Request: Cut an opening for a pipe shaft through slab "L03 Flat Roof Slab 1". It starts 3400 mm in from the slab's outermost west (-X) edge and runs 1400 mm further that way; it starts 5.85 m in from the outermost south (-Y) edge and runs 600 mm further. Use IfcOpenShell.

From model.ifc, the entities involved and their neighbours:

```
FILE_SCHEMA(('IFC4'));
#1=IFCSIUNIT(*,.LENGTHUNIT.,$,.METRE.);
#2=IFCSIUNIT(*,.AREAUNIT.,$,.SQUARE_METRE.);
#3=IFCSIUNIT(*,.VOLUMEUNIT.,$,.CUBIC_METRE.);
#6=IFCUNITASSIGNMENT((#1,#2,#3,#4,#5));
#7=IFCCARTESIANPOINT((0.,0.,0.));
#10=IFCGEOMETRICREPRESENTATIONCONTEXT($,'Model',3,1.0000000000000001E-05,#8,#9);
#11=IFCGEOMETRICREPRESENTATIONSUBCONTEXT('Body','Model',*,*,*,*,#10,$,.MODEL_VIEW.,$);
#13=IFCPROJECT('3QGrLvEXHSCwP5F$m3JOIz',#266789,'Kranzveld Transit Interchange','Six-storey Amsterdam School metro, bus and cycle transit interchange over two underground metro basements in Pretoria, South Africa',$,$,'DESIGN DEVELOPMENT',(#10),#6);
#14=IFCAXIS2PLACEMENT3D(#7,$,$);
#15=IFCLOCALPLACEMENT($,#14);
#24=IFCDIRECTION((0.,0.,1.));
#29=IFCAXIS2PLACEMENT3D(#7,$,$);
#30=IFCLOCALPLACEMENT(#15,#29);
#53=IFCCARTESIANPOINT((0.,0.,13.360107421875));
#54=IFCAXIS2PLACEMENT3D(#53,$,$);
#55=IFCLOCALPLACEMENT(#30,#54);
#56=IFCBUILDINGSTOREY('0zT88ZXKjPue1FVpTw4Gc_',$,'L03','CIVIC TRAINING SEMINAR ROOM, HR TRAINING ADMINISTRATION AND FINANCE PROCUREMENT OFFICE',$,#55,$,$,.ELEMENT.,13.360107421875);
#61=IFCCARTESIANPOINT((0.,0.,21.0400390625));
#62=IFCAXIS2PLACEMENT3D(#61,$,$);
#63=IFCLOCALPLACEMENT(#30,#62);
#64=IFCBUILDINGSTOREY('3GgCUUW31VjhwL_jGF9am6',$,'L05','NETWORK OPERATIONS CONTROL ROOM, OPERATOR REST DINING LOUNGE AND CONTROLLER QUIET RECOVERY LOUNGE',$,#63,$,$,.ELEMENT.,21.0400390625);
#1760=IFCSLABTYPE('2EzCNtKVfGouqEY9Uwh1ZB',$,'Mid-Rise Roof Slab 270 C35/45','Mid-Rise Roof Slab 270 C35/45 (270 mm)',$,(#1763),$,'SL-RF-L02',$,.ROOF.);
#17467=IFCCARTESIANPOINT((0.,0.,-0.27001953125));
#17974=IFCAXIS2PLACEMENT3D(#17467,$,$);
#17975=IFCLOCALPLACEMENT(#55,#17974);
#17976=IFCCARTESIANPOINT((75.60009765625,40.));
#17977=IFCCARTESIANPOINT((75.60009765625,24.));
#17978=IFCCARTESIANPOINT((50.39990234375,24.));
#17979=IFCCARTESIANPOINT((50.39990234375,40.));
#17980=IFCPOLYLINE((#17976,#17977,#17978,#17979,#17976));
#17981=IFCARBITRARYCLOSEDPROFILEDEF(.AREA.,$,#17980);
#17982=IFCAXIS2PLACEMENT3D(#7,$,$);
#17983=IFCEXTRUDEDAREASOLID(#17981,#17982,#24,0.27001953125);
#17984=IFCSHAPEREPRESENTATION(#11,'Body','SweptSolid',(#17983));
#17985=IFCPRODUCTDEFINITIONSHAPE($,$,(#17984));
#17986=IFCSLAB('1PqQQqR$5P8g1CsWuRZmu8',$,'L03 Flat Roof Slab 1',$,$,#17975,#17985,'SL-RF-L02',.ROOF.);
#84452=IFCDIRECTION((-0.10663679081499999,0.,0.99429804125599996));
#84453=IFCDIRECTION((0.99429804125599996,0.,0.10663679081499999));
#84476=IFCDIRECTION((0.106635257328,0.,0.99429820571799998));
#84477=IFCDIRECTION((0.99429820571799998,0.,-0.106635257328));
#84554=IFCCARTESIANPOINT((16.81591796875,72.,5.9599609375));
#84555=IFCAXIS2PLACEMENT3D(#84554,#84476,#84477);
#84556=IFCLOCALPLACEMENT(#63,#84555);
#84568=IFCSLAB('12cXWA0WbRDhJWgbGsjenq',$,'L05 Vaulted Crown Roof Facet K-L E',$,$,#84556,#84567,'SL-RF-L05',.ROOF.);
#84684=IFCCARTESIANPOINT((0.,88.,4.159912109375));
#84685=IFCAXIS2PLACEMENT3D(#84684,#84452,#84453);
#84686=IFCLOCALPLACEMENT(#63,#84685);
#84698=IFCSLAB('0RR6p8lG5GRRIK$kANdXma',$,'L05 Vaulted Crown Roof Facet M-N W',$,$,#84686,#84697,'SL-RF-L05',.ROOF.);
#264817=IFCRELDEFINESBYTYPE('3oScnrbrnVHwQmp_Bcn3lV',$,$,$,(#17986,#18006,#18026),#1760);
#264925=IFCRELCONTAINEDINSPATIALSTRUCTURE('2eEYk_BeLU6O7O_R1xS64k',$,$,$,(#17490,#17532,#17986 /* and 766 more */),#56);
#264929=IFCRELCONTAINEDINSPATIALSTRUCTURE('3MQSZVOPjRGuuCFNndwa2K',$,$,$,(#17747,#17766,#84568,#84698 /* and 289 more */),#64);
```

```python
import numpy as np
import ifcopenshell
import ifcopenshell.api.feature
import ifcopenshell.api.geometry
import ifcopenshell.api.root
import ifcopenshell.geom
import ifcopenshell.util.placement
import ifcopenshell.util.representation
import ifcopenshell.util.shape
import ifcopenshell.util.unit

model = ifcopenshell.open("model.ifc")
unit_scale = ifcopenshell.util.unit.calculate_unit_scale(model)
settings = ifcopenshell.geom.settings()


def volume(element):
    """Net volume in cubic metres, openings subtracted."""
    shape = ifcopenshell.geom.create_shape(settings, element)
    return ifcopenshell.util.shape.get_volume(shape.geometry)


slab = model.by_guid("1PqQQqR$5P8g1CsWuRZmu8")
before = volume(slab)

# Extent in the slab's own axes, in metres. The edges named are its -X and -Y sides.
slab_shape = ifcopenshell.geom.create_shape(settings, slab)
vertices = ifcopenshell.util.shape.get_vertices(slab_shape.geometry)
x_min, y_min, bottom = vertices.min(axis=0)
top = vertices[:, 2].max()

opening = ifcopenshell.api.root.create_entity(model, ifc_class="IfcOpeningElement", name="Pipe shaft opening", predefined_type="OPENING")
context = ifcopenshell.util.representation.get_context(model, "Model", "Body", "MODEL_VIEW")
width, depth = 1.4, 0.6
outline = [(0.0, 0.0), (width, 0.0), (width, depth), (0.0, depth), (0.0, 0.0)]
# Overshoot both faces by 50 mm so the cut is clean.
shape = ifcopenshell.api.geometry.add_slab_representation(
    model, context=context, depth=top - bottom + 0.1, polyline=outline
)
ifcopenshell.api.geometry.assign_representation(model, product=opening, representation=shape)

matrix = ifcopenshell.util.placement.get_local_placement(slab.ObjectPlacement)
matrix[:, 3] = matrix @ np.append(np.array([x_min + 3.4, y_min + 5.85, bottom - 0.05]) / unit_scale, 1.0)
ifcopenshell.api.geometry.edit_object_placement(model, product=opening, matrix=matrix, is_si=False)
ifcopenshell.api.feature.add_feature(model, feature=opening, element=slab)

after = volume(slab)

print(f"slab volume {before:.3f} -> {after:.3f} m3")

model.write("model_rev.ifc")
```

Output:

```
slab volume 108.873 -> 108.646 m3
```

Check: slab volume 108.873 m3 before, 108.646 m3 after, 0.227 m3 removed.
